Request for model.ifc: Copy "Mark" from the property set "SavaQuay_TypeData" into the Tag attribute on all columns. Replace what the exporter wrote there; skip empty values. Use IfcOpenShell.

First a look at what the model holds.

```python
import ifcopenshell
import ifcopenshell.util.element

model = ifcopenshell.open("model.ifc")
print(model.schema)
columns = model.by_type("IfcColumn")
print(len(columns), "columns")
for e in columns[:8]:
    source = ifcopenshell.util.element.get_pset(e, "SavaQuay_TypeData", "Mark")
    target = e.Tag
    print(e.id(), repr(source), repr(target), sep=" | ")
```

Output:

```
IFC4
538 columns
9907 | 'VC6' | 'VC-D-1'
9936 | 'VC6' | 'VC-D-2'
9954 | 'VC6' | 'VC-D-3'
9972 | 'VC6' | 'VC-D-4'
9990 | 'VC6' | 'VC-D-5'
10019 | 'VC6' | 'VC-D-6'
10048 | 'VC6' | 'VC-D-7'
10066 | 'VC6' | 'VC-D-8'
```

```python
import ifcopenshell
import ifcopenshell.util.element

model = ifcopenshell.open("model.ifc")

count = 0
for e in model.by_type("IfcColumn"):
    value = ifcopenshell.util.element.get_pset(e, "SavaQuay_TypeData", "Mark")
    current = e.Tag
    if not value or not value.strip() or current == value:
        continue
    e.Tag = value
    count += 1

print(count, "columns updated")

model.write("model_updated.ifc")
```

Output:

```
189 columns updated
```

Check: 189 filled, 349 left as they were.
